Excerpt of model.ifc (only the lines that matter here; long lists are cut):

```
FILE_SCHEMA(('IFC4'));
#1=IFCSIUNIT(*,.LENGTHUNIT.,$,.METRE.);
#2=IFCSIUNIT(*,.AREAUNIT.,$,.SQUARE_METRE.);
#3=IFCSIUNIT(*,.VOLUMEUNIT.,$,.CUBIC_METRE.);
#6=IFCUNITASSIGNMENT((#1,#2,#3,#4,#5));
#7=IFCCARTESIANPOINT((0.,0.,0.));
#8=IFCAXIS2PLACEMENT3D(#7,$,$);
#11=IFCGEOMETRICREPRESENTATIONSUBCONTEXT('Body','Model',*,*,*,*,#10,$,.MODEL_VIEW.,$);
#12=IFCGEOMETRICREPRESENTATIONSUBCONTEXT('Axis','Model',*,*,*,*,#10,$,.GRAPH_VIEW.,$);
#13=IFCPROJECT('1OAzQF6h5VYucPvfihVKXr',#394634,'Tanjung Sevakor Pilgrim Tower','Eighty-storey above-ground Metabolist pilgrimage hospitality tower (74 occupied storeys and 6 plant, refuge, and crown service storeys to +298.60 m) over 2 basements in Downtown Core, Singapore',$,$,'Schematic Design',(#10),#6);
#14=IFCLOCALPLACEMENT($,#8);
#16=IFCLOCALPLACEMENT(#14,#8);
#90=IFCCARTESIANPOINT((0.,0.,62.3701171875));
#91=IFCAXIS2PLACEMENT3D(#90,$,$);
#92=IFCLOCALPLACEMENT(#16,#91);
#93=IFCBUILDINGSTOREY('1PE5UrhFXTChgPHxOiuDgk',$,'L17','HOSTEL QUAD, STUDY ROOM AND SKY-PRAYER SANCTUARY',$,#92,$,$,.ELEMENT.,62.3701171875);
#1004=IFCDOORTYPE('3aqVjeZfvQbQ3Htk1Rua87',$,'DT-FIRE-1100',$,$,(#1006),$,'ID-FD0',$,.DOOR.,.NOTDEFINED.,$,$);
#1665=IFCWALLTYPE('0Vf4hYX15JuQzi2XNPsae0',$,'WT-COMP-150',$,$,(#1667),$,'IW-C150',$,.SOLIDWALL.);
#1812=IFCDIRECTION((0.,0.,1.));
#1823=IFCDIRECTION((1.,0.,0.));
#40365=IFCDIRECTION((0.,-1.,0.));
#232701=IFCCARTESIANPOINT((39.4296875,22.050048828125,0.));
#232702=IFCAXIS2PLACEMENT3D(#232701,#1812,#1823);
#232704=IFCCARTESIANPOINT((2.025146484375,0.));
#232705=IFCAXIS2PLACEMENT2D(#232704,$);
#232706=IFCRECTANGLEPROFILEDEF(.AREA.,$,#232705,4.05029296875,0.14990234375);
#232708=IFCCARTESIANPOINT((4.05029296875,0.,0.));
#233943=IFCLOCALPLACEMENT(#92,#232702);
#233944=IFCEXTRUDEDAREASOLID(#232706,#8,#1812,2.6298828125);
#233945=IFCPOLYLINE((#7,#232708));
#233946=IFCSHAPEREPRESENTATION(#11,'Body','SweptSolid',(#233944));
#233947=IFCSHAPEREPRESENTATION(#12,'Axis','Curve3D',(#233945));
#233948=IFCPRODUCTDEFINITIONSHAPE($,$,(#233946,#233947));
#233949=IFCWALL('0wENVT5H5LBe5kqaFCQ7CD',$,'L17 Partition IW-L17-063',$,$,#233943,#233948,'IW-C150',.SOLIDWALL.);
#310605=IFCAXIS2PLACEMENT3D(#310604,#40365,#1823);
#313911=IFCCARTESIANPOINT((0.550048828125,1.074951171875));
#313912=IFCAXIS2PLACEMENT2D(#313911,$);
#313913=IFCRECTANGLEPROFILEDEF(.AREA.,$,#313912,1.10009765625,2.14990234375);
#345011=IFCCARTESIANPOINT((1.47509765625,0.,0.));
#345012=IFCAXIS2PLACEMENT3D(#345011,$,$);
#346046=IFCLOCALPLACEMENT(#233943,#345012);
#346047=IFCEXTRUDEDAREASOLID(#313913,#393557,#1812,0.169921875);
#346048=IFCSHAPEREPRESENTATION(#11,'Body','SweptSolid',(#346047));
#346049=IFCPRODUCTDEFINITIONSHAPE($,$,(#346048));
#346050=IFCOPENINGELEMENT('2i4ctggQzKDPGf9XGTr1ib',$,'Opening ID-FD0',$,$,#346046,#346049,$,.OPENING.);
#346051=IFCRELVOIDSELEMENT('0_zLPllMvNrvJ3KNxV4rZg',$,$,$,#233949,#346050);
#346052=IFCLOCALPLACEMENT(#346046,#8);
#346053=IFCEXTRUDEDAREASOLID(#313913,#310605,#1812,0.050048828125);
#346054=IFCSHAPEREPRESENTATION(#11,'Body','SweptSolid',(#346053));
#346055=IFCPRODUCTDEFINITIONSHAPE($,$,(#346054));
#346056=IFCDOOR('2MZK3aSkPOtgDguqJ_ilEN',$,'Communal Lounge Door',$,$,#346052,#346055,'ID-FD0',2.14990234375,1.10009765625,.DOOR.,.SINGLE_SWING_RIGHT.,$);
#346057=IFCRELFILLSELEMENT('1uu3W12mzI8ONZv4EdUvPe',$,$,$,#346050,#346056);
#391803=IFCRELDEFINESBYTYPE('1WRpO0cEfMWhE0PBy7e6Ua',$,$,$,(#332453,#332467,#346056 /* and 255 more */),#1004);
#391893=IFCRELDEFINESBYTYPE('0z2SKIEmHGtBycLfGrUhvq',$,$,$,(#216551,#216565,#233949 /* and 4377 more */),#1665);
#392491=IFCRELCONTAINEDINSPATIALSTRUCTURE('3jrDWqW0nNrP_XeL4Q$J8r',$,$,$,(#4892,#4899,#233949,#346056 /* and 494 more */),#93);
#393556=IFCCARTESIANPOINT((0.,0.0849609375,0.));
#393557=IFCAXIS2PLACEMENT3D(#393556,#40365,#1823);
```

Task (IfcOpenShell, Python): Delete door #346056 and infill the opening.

```python
import ifcopenshell
import ifcopenshell.api.feature
import ifcopenshell.api.root
import ifcopenshell.geom
import ifcopenshell.util.shape

model = ifcopenshell.open("model.ifc")
settings = ifcopenshell.geom.settings()


def volume(element):
    """Net volume in cubic metres, openings subtracted."""
    shape = ifcopenshell.geom.create_shape(settings, element)
    return ifcopenshell.util.shape.get_volume(shape.geometry)


door = model.by_id(346056)
opening = door.FillsVoids[0].RelatingOpeningElement
wall = opening.VoidsElements[0].RelatingBuildingElement
before = volume(wall)

ifcopenshell.api.root.remove_product(model, product=door)
ifcopenshell.api.feature.remove_feature(model, feature=opening)

after = volume(wall)

print(f"wall volume {before:.3f} -> {after:.3f} m3")

model.write("model_updated.ifc")
```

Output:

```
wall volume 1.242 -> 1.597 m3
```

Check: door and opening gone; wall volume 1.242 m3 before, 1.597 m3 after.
